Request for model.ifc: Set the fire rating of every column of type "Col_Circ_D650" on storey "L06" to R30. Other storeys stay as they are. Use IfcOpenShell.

First a look at what the model holds.

```python
import ifcopenshell
import ifcopenshell.util.element

model = ifcopenshell.open("model.ifc")
print(model.schema)
storey = next(s for s in model.by_type("IfcBuildingStorey") if s.Name == "L06")
columns = [e for e in ifcopenshell.util.element.get_decomposition(storey) if e.is_a("IfcColumn")]
seen = {}
for e in columns:
    element_type = ifcopenshell.util.element.get_type(e)
    key = (element_type.Name if element_type != e and element_type else None, ifcopenshell.util.element.get_pset(e, "Pset_ColumnCommon", "FireRating"))
    seen[key] = seen.get(key, 0) + 1
for (name, value), count in sorted(seen.items(), key=str):
    print(count, "x", name, "|", value)
```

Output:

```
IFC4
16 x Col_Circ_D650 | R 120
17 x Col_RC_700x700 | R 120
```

```python
import ifcopenshell
import ifcopenshell.api.pset
import ifcopenshell.util.element

model = ifcopenshell.open("model.ifc")

storey = next(s for s in model.by_type("IfcBuildingStorey") if s.Name == "L06")
columns = [e for e in ifcopenshell.util.element.get_decomposition(storey) if e.is_a("IfcColumn")]

count = 0
for e in columns:
    element_type = ifcopenshell.util.element.get_type(e)
    if element_type in (None, e) or element_type.Name != "Col_Circ_D650":
        continue
    # add_pset returns the element's existing set when there is one.
    pset = ifcopenshell.api.pset.add_pset(model, product=e, name="Pset_ColumnCommon")
    ifcopenshell.api.pset.edit_pset(model, pset=pset, properties={"FireRating": "R30"})
    count += 1

print(count, "columns updated")

model.write("model_edited.ifc")
```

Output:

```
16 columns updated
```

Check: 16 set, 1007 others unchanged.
